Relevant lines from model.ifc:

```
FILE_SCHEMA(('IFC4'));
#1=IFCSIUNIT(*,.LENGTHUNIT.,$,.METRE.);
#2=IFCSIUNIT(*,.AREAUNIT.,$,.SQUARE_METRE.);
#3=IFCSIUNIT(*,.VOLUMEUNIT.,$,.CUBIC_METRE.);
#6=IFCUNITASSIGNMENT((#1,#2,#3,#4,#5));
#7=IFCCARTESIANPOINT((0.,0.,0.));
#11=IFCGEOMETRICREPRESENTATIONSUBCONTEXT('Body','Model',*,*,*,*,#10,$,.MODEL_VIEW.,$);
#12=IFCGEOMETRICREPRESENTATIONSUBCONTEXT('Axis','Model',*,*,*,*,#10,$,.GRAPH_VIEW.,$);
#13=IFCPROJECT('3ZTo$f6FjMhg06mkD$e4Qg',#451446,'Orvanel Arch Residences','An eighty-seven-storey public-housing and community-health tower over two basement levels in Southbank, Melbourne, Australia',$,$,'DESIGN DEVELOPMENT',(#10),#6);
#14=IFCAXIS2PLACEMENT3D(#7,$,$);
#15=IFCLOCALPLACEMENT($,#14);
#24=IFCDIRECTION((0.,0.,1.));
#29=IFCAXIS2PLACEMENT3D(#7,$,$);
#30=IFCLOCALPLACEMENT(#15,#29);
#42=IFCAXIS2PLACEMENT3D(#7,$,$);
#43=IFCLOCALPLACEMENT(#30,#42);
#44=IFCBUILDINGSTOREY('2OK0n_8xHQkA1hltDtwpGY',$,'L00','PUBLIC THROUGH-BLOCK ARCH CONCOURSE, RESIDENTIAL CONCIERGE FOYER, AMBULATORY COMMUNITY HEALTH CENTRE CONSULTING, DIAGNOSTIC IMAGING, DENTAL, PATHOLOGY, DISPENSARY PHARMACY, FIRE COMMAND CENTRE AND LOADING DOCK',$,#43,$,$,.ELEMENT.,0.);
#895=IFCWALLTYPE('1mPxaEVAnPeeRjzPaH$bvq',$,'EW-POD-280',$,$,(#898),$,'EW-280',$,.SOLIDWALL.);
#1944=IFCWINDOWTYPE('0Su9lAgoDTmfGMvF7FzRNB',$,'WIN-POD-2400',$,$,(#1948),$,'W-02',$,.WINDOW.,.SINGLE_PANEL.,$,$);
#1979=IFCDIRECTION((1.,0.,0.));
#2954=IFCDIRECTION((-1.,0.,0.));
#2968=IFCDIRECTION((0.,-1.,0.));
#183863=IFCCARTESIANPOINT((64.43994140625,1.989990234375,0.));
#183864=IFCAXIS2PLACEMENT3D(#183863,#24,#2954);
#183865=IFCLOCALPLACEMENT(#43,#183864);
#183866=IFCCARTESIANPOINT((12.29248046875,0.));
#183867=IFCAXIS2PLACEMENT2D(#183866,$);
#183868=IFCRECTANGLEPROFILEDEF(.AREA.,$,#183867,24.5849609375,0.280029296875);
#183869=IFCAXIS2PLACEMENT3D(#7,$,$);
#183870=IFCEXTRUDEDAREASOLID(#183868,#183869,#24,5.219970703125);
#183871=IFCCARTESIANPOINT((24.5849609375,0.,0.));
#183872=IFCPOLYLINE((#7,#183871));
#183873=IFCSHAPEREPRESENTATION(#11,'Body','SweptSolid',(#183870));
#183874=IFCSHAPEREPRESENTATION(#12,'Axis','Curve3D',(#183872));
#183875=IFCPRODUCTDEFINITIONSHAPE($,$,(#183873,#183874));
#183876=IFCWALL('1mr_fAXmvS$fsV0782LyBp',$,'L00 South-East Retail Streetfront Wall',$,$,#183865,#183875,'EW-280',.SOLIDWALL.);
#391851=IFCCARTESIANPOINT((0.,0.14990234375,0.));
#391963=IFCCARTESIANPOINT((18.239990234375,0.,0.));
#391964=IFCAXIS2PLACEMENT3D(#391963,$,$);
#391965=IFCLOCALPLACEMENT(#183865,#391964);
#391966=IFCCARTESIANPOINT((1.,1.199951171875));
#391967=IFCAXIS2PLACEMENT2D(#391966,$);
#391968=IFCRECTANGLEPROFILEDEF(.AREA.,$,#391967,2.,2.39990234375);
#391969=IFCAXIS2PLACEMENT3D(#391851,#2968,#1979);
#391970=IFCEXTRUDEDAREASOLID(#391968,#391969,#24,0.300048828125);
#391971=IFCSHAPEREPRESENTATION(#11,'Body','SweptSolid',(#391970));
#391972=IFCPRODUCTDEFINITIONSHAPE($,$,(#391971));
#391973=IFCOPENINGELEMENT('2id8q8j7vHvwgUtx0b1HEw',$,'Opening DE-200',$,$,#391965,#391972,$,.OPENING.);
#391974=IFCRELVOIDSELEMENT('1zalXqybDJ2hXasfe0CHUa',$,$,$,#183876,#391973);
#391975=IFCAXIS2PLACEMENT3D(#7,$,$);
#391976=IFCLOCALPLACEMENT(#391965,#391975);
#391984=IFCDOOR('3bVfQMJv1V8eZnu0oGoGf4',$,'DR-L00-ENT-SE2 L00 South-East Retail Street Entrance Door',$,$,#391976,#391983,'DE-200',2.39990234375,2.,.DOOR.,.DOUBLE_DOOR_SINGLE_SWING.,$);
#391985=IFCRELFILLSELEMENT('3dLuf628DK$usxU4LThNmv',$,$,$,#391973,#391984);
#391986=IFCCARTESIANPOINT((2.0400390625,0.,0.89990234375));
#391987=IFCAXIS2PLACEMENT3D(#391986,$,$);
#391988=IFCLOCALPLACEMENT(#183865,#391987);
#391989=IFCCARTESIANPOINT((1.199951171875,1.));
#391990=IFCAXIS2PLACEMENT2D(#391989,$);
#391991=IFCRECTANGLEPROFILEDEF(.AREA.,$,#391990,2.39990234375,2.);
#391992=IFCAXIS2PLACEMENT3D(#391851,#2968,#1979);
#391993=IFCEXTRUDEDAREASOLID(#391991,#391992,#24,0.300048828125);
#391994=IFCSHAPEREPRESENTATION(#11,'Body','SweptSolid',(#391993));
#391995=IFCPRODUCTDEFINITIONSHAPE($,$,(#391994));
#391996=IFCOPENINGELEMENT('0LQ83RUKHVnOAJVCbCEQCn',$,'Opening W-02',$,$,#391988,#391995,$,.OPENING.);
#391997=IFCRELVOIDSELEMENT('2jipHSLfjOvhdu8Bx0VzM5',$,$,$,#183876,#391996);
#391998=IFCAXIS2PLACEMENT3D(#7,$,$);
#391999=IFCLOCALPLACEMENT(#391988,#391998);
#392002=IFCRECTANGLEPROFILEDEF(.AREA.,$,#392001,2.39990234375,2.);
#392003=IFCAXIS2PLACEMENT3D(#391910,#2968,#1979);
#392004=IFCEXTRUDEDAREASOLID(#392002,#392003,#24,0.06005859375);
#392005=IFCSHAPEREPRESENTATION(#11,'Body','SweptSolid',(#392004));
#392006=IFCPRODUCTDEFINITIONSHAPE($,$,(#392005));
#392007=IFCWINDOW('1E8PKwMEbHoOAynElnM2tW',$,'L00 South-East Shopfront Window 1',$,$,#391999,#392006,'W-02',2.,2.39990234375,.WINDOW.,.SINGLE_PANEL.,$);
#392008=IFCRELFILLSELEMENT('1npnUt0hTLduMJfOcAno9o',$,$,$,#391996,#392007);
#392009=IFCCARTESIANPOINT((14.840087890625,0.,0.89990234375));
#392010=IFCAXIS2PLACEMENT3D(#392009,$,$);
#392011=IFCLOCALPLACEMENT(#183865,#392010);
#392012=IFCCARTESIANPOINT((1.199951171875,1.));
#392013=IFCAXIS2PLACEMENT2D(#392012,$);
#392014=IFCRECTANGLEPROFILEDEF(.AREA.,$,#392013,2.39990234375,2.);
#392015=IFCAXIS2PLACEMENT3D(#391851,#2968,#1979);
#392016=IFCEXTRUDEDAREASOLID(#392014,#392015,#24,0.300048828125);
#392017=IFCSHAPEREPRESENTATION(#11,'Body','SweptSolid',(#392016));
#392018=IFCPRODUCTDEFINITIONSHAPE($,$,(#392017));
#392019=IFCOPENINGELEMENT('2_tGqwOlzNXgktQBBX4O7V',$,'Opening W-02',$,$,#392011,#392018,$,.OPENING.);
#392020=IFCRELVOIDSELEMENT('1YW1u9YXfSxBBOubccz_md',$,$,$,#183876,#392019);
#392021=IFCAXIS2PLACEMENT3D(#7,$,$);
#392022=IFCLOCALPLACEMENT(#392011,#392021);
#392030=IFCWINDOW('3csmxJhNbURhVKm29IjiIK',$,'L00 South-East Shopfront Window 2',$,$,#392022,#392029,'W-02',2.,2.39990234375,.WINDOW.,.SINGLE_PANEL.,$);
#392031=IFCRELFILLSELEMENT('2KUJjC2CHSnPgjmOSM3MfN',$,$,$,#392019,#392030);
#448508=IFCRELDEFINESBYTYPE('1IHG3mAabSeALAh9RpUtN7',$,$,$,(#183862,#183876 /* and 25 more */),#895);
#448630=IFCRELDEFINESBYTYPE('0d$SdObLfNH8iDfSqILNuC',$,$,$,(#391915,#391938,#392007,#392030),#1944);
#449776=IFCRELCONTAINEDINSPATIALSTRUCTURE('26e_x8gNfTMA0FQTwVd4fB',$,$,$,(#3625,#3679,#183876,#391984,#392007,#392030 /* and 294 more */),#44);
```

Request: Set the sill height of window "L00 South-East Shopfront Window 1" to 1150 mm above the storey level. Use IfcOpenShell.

```python
import numpy as np
import ifcopenshell
import ifcopenshell.api.geometry
import ifcopenshell.geom
import ifcopenshell.util.element
import ifcopenshell.util.placement
import ifcopenshell.util.shape
import ifcopenshell.util.unit

model = ifcopenshell.open("model.ifc")
unit_scale = ifcopenshell.util.unit.calculate_unit_scale(model)

window = model.by_guid("1E8PKwMEbHoOAynElnM2tW")
opening = window.FillsVoids[0].RelatingOpeningElement
storey = ifcopenshell.util.element.get_container(window, ifc_class="IfcBuildingStorey")
level = ifcopenshell.util.placement.get_local_placement(storey.ObjectPlacement)[2, 3]

# The opening's origin need not be at the sill, so measure its lowest point.
shape = ifcopenshell.geom.create_shape(ifcopenshell.geom.settings(), opening)
bottom = ifcopenshell.util.shape.get_shape_bottom_elevation(shape, shape.geometry) / unit_scale
dz = level + 1.15 - bottom

shift = np.array([0.0, 0.0, dz])
# The window is placed relative to its opening, so it follows when the opening moves.
matrix = ifcopenshell.util.placement.get_local_placement(opening.ObjectPlacement)
matrix[:3, 3] += shift
ifcopenshell.api.geometry.edit_object_placement(
    model, product=opening, matrix=matrix, is_si=False, should_transform_children=True
)

print(f"moved by {dz * unit_scale:+.3f} m")

model.write("model-out.ifc")
```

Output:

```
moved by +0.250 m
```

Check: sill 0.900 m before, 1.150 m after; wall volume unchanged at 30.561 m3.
